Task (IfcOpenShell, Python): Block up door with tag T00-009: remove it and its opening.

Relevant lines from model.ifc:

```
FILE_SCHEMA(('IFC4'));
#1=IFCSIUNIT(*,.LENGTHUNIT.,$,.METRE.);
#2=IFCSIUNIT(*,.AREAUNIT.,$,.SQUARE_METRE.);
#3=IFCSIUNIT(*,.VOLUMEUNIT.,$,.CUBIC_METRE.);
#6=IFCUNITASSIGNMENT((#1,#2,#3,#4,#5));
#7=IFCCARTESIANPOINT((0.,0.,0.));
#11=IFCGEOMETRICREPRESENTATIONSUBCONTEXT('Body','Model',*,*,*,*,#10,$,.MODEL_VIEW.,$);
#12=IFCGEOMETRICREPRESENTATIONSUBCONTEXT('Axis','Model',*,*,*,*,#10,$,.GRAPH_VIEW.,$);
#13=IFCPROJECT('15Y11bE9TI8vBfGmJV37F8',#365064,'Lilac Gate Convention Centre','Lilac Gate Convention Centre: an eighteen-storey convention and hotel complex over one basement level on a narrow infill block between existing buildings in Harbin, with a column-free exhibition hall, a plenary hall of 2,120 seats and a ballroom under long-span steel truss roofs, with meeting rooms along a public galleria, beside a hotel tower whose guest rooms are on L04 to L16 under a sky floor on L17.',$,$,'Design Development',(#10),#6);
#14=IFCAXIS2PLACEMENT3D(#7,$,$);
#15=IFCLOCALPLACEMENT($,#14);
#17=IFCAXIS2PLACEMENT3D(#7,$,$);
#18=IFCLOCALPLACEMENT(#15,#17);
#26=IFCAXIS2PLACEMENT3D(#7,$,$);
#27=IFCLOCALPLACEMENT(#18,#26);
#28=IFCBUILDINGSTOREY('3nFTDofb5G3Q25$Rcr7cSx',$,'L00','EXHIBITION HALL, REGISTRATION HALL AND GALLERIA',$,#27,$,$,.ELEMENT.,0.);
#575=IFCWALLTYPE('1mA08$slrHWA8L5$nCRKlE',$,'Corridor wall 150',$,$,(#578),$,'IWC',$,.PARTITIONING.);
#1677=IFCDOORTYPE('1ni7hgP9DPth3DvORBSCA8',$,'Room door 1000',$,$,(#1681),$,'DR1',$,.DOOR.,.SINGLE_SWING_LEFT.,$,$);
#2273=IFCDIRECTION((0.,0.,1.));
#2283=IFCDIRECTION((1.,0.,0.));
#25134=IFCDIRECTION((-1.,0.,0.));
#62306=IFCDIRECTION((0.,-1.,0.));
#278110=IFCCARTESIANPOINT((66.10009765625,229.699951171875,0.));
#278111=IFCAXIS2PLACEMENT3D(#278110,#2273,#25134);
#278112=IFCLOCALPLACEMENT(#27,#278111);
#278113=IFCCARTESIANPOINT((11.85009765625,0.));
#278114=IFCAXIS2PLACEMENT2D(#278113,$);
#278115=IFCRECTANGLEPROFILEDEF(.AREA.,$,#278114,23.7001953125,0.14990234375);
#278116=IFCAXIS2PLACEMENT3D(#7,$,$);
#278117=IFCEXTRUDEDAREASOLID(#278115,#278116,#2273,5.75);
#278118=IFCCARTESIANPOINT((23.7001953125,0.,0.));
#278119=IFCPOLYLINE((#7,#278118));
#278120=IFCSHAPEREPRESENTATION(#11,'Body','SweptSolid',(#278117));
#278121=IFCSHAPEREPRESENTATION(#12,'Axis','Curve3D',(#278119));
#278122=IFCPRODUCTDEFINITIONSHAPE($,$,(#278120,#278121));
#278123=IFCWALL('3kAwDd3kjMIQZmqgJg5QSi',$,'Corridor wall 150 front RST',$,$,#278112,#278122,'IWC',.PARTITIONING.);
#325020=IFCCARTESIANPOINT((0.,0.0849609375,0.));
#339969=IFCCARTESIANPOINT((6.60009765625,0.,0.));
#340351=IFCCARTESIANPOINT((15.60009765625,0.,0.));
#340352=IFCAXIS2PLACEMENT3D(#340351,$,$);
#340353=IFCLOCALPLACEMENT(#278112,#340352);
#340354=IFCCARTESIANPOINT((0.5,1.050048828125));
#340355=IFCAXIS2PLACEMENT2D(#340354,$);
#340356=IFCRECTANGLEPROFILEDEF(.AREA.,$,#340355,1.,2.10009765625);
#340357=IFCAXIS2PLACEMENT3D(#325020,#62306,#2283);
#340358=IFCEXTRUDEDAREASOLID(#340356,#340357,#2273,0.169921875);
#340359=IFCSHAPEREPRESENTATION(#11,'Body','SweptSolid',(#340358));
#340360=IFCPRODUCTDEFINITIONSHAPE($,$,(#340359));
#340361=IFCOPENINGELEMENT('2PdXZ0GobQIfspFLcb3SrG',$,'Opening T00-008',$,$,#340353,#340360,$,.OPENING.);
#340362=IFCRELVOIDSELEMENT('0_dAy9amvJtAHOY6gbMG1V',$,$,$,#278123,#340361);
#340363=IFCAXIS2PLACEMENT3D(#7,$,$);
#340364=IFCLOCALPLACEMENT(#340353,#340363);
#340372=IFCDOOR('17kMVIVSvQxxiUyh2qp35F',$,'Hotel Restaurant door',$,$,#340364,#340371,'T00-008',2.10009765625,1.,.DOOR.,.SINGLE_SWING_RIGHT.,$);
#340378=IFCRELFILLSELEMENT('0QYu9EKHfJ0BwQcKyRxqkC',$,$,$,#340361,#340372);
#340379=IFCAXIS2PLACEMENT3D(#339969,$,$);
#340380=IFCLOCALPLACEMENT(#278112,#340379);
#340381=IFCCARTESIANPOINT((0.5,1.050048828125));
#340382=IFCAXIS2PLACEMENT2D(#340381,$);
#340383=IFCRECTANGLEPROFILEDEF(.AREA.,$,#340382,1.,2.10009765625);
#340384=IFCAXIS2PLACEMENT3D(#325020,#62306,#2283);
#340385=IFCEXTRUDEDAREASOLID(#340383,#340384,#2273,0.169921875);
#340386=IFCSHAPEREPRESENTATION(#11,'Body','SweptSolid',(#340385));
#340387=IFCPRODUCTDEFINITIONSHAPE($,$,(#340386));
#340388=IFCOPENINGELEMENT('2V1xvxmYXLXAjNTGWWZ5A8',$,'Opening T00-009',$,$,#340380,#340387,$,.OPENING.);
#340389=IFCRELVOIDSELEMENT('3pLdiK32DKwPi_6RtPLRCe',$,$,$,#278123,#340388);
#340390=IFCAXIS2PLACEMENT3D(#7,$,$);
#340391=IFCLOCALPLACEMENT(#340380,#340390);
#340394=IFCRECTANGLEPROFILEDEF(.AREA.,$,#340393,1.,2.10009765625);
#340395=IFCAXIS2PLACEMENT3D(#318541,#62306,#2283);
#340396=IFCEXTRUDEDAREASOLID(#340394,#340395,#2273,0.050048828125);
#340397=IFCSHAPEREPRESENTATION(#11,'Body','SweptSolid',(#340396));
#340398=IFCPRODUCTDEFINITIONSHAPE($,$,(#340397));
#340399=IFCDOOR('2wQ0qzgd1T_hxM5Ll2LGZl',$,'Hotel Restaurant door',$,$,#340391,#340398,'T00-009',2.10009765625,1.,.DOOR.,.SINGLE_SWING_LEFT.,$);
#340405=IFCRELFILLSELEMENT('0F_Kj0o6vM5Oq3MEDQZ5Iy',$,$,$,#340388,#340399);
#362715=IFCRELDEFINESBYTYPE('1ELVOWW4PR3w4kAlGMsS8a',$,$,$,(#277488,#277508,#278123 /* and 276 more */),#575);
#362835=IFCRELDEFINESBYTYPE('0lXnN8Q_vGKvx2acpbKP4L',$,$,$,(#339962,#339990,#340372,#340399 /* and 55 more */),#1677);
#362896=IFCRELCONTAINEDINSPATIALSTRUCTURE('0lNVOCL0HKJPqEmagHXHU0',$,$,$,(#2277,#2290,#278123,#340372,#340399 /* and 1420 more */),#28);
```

```python
import ifcopenshell
import ifcopenshell.api.feature
import ifcopenshell.api.root
import ifcopenshell.geom
import ifcopenshell.util.shape

model = ifcopenshell.open("model.ifc")
settings = ifcopenshell.geom.settings()


def volume(element):
    """Net volume in cubic metres, openings subtracted."""
    shape = ifcopenshell.geom.create_shape(settings, element)
    return ifcopenshell.util.shape.get_volume(shape.geometry)


door = model.by_id(340399)
opening = door.FillsVoids[0].RelatingOpeningElement
wall = opening.VoidsElements[0].RelatingBuildingElement
before = volume(wall)

ifcopenshell.api.root.remove_product(model, product=door)
ifcopenshell.api.feature.remove_feature(model, feature=opening)

after = volume(wall)

print(f"wall volume {before:.3f} -> {after:.3f} m3")

model.write("model_rev.ifc")
```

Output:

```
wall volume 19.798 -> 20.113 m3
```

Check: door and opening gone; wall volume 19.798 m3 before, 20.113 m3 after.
